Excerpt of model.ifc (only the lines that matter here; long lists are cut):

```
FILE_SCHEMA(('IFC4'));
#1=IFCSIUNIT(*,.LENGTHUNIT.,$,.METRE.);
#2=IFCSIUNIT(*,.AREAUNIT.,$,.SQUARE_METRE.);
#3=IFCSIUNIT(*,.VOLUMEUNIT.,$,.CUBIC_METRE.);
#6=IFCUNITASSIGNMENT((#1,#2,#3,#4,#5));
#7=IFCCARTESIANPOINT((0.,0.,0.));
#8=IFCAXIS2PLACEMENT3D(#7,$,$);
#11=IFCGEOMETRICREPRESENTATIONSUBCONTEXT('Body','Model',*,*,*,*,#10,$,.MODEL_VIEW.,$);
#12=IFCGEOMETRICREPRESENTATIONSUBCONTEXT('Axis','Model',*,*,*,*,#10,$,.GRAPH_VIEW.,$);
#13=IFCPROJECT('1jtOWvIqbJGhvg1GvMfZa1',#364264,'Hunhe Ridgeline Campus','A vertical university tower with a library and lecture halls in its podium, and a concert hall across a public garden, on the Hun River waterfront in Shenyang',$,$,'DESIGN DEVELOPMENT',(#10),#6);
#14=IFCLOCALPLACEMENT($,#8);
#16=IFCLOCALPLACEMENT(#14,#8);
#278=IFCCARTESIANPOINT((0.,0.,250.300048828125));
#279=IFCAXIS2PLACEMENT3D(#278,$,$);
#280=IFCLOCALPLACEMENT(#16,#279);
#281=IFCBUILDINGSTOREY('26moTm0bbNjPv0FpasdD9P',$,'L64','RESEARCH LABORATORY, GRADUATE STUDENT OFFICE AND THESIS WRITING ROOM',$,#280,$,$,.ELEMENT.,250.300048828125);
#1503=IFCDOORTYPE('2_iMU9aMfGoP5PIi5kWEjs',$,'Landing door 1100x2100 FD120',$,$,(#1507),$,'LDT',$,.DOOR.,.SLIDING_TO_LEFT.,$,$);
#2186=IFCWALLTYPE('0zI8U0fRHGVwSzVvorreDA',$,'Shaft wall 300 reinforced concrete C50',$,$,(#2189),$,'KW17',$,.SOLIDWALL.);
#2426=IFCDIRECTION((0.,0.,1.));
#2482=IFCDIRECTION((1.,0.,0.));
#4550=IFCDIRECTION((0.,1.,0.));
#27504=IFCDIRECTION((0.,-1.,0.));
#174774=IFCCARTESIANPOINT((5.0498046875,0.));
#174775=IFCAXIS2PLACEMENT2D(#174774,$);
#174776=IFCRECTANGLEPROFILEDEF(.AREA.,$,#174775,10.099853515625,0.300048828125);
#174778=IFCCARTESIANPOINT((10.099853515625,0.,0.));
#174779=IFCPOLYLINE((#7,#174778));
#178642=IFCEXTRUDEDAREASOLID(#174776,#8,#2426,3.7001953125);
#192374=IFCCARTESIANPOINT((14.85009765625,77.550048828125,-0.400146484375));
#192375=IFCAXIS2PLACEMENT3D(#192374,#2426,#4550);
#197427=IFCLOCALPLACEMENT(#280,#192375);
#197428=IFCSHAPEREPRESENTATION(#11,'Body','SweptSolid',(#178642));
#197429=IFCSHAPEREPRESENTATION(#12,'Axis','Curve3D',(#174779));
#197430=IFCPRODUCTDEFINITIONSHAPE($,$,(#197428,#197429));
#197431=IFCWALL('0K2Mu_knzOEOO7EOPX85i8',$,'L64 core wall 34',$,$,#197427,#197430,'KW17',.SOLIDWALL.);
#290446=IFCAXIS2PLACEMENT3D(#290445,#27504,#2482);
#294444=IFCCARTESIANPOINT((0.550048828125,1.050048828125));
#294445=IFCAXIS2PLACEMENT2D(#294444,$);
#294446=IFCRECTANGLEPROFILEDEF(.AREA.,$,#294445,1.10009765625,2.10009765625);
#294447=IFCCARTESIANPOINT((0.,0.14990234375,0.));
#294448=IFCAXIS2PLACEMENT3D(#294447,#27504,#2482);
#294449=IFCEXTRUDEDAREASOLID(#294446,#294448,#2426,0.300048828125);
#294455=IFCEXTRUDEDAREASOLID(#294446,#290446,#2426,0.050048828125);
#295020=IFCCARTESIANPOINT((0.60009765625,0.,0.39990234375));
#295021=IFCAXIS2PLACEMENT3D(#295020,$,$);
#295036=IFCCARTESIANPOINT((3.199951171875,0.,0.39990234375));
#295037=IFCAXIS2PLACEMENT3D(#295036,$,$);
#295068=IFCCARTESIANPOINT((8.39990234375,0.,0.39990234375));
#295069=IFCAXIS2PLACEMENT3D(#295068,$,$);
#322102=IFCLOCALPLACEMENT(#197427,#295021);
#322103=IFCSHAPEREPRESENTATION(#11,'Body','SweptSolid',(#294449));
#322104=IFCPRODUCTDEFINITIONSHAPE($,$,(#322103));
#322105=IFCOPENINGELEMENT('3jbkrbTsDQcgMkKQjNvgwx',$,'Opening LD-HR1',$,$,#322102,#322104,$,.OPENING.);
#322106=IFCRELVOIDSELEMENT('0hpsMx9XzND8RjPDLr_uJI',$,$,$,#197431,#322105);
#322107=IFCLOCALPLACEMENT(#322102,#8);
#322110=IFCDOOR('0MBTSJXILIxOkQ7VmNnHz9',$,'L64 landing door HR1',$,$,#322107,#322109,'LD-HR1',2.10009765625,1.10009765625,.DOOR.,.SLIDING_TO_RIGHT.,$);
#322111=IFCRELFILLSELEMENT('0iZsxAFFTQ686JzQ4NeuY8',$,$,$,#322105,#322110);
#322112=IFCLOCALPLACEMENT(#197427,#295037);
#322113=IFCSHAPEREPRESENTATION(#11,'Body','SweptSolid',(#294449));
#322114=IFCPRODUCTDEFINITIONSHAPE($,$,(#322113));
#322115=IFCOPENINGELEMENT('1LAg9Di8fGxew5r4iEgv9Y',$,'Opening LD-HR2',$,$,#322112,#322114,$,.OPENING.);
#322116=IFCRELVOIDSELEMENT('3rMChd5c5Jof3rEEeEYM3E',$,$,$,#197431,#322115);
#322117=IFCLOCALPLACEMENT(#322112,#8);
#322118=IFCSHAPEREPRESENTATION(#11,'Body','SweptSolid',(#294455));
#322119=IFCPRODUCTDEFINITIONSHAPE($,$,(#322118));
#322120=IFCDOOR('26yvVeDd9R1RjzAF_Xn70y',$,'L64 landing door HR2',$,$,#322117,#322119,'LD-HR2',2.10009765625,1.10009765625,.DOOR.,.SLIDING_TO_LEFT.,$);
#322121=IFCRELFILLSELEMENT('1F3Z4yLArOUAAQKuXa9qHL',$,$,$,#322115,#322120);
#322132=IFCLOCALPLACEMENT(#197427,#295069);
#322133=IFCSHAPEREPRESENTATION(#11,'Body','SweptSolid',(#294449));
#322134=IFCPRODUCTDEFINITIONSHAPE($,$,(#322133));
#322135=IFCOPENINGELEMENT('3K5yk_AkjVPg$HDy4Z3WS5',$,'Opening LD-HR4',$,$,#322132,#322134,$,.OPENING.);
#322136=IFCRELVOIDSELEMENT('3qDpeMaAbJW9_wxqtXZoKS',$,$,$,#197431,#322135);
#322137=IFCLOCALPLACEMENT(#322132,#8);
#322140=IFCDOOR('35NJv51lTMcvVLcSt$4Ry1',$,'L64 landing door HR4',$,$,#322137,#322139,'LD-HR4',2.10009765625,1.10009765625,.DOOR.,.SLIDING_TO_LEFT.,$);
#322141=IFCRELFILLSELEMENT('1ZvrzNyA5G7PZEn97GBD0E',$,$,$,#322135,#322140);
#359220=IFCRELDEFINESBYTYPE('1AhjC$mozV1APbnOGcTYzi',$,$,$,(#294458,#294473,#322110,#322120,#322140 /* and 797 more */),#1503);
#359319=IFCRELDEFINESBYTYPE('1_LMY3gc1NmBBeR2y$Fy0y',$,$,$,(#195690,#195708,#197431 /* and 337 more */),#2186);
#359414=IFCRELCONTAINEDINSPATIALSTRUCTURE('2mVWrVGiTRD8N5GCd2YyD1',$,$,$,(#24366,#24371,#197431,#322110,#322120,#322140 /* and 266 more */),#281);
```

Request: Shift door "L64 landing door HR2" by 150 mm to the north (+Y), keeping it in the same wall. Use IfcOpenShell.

```python
import ifcopenshell
import ifcopenshell.api.geometry
import ifcopenshell.util.placement
import ifcopenshell.util.unit

model = ifcopenshell.open("model.ifc")
unit_scale = ifcopenshell.util.unit.calculate_unit_scale(model)

door = model.by_guid("26yvVeDd9R1RjzAF_Xn70y")
opening = door.FillsVoids[0].RelatingOpeningElement
wall = opening.VoidsElements[0].RelatingBuildingElement

wall_matrix = ifcopenshell.util.placement.get_local_placement(wall.ObjectPlacement)
shift = wall_matrix[:3, 0] * 0.15 / unit_scale
before = ifcopenshell.util.placement.get_local_placement(door.ObjectPlacement)[:3, 3].copy()

# The door is placed relative to its opening, so it follows when the opening moves.
matrix = ifcopenshell.util.placement.get_local_placement(opening.ObjectPlacement)
matrix[:3, 3] += shift
ifcopenshell.api.geometry.edit_object_placement(
    model, product=opening, matrix=matrix, is_si=False, should_transform_children=True
)

after = ifcopenshell.util.placement.get_local_placement(door.ObjectPlacement)[:3, 3]
print("door moved by", (after - before).round(3) + 0.0)

model.write("model_edited.ifc")
```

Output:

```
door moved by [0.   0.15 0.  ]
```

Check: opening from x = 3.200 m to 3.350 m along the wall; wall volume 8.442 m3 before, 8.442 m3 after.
